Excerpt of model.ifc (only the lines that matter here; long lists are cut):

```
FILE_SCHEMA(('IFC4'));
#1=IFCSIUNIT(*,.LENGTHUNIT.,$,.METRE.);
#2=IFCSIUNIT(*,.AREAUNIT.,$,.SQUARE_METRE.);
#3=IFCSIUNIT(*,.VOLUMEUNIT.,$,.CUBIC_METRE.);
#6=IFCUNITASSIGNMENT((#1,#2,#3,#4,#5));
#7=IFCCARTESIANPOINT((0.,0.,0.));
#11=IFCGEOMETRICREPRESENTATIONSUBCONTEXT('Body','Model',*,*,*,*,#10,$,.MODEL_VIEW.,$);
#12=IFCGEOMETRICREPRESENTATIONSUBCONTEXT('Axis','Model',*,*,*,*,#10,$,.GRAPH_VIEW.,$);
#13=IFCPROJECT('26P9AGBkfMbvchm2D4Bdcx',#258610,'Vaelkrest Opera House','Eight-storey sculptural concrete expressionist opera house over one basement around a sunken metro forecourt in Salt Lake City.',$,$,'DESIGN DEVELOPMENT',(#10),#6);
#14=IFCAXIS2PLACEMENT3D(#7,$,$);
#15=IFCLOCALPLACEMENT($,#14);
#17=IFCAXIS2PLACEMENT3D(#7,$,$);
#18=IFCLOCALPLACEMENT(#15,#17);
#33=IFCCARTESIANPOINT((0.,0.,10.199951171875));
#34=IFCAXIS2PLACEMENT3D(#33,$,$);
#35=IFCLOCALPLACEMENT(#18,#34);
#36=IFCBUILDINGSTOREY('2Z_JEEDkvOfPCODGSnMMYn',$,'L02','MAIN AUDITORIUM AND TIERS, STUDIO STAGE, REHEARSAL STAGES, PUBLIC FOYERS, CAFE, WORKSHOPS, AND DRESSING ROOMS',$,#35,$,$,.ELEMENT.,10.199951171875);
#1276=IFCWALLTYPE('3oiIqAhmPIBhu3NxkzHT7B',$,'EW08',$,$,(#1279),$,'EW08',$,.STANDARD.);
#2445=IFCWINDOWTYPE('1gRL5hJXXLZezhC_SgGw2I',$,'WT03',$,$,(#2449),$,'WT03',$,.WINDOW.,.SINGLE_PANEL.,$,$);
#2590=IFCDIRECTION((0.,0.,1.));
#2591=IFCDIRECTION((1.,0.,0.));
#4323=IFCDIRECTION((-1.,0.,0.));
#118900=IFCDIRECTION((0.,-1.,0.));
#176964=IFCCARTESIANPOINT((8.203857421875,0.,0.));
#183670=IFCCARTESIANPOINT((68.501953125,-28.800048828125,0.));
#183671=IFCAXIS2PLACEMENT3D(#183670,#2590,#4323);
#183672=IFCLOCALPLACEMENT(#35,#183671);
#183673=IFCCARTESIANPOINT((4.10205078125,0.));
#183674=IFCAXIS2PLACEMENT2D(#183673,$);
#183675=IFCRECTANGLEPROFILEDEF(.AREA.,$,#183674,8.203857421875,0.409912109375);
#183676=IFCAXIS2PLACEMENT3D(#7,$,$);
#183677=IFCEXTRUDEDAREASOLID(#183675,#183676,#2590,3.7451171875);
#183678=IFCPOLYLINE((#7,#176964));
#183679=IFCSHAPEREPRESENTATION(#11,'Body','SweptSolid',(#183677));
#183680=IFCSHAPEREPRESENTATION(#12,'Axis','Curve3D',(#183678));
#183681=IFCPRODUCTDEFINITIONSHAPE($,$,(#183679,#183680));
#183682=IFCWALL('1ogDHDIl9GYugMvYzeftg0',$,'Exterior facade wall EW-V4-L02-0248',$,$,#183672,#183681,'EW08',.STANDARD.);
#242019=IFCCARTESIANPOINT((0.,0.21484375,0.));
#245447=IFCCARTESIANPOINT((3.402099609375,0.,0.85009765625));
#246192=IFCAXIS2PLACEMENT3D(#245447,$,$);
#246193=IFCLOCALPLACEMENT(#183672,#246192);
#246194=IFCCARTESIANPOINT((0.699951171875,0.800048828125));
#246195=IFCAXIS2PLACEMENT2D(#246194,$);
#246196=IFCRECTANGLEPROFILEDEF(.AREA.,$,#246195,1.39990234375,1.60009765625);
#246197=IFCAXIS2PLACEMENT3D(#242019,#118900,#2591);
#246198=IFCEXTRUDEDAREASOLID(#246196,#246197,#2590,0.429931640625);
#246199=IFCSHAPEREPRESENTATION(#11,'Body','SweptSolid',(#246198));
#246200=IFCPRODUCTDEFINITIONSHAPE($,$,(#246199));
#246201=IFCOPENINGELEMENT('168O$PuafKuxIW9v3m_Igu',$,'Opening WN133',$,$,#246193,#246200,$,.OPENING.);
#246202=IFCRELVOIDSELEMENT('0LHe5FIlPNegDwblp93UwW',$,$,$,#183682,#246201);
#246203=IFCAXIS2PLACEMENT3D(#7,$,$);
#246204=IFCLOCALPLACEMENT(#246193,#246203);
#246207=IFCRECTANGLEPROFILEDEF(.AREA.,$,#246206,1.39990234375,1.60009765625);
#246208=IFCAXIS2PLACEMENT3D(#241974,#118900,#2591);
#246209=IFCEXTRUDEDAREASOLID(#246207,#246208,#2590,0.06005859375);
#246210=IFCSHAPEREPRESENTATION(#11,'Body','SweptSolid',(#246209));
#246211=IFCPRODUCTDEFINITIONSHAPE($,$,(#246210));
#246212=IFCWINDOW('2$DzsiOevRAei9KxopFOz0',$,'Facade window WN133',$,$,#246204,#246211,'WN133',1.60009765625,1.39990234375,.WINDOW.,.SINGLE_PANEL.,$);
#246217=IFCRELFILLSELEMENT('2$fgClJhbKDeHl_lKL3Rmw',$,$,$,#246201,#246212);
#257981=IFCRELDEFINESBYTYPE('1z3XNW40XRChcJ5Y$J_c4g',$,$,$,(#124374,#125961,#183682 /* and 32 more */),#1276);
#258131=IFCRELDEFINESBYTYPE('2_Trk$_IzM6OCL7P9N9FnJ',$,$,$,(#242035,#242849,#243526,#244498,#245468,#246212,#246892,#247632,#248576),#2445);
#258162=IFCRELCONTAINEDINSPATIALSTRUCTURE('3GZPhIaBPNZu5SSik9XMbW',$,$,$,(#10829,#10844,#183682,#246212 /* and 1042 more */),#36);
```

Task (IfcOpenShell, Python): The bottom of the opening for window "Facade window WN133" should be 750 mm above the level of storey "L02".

```python
import numpy as np
import ifcopenshell
import ifcopenshell.api.geometry
import ifcopenshell.geom
import ifcopenshell.util.element
import ifcopenshell.util.placement
import ifcopenshell.util.shape
import ifcopenshell.util.unit

model = ifcopenshell.open("model.ifc")
unit_scale = ifcopenshell.util.unit.calculate_unit_scale(model)

window = model.by_guid("2$DzsiOevRAei9KxopFOz0")
opening = window.FillsVoids[0].RelatingOpeningElement
storey = ifcopenshell.util.element.get_container(window, ifc_class="IfcBuildingStorey")
level = ifcopenshell.util.placement.get_local_placement(storey.ObjectPlacement)[2, 3]

# The opening's origin need not be at the sill, so measure its lowest point.
shape = ifcopenshell.geom.create_shape(ifcopenshell.geom.settings(), opening)
bottom = ifcopenshell.util.shape.get_shape_bottom_elevation(shape, shape.geometry) / unit_scale
dz = level + 0.75 / unit_scale - bottom

shift = np.array([0.0, 0.0, dz])
# The window is placed relative to its opening, so it follows when the opening moves.
matrix = ifcopenshell.util.placement.get_local_placement(opening.ObjectPlacement)
matrix[:3, 3] += shift
ifcopenshell.api.geometry.edit_object_placement(
    model, product=opening, matrix=matrix, is_si=False, should_transform_children=True
)

print(f"moved by {dz * unit_scale:+.3f} m")

model.write("model_rev.ifc")
```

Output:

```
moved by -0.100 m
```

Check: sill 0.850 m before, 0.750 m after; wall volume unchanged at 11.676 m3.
